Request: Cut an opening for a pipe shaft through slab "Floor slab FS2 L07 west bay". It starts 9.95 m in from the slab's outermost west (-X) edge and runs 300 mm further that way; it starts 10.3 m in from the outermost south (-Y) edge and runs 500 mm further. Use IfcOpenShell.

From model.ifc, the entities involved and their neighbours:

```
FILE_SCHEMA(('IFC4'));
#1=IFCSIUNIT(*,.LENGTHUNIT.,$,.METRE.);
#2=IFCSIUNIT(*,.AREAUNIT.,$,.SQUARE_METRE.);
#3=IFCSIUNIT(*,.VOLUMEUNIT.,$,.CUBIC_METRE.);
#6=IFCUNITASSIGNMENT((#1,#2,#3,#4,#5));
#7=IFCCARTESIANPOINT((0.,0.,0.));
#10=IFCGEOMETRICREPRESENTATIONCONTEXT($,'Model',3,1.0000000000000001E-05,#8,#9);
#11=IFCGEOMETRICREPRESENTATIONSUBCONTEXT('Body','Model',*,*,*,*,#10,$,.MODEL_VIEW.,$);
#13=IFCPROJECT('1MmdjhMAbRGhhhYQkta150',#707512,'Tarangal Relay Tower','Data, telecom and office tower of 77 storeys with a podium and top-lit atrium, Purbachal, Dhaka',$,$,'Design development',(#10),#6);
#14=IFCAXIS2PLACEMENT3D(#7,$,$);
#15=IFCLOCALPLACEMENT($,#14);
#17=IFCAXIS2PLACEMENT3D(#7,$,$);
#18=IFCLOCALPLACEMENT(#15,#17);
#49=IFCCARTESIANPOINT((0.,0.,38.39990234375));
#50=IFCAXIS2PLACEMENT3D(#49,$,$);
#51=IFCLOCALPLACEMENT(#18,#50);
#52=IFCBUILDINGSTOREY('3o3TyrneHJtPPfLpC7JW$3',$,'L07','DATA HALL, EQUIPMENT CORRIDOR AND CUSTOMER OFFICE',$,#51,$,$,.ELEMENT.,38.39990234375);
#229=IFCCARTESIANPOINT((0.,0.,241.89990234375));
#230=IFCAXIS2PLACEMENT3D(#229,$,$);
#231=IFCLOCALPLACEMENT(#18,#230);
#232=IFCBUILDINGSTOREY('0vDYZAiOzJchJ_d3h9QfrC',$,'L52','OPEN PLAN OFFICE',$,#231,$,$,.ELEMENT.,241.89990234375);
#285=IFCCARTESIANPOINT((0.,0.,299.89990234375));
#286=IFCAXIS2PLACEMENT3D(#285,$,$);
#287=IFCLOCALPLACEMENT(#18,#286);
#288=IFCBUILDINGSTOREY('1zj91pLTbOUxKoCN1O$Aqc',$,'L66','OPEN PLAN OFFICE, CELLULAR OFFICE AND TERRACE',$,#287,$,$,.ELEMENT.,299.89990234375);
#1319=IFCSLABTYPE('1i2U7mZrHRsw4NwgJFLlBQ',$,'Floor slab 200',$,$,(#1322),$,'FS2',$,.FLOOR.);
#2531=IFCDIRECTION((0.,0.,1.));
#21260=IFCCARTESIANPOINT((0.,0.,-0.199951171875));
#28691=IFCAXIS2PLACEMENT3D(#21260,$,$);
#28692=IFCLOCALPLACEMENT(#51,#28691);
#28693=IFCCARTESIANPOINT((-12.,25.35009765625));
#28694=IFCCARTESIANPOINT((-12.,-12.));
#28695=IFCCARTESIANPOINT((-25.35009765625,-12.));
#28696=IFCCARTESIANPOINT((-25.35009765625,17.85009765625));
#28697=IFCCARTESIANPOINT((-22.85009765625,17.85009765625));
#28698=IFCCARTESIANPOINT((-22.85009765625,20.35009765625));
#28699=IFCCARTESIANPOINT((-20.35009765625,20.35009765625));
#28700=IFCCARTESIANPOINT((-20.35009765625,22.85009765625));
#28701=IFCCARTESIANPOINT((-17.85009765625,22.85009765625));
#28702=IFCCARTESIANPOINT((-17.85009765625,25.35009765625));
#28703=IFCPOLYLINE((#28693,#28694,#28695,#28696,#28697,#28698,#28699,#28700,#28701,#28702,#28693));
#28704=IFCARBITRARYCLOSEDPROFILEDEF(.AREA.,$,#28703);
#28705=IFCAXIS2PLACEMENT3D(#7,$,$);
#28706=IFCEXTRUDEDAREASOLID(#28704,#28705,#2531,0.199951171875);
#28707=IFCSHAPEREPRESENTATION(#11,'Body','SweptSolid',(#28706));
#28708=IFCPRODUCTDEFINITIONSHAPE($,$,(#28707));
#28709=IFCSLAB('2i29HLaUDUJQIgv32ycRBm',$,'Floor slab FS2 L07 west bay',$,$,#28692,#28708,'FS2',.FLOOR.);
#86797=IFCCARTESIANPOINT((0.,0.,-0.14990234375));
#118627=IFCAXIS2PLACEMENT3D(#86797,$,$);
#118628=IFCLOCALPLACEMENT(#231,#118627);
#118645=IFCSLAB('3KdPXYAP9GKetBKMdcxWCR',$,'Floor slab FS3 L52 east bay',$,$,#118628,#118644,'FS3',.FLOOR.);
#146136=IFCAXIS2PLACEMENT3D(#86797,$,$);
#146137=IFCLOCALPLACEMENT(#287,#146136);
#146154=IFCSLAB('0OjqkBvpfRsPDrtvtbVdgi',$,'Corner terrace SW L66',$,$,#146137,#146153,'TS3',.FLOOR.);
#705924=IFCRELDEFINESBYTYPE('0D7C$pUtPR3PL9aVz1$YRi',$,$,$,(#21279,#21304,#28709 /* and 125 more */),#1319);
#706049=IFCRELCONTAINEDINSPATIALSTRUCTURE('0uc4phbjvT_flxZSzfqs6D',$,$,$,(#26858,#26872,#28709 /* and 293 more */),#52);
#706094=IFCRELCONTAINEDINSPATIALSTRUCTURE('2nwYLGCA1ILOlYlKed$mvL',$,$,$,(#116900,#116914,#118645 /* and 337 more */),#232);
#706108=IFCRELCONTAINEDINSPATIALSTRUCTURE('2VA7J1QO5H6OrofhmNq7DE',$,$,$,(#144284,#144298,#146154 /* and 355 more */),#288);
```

```python
import numpy as np
import ifcopenshell
import ifcopenshell.api.feature
import ifcopenshell.api.geometry
import ifcopenshell.api.root
import ifcopenshell.geom
import ifcopenshell.util.placement
import ifcopenshell.util.representation
import ifcopenshell.util.shape
import ifcopenshell.util.unit

model = ifcopenshell.open("model.ifc")
unit_scale = ifcopenshell.util.unit.calculate_unit_scale(model)
settings = ifcopenshell.geom.settings()


def volume(element):
    """Net volume in cubic metres, openings subtracted."""
    shape = ifcopenshell.geom.create_shape(settings, element)
    return ifcopenshell.util.shape.get_volume(shape.geometry)


slab = model.by_guid("2i29HLaUDUJQIgv32ycRBm")
before = volume(slab)

# Extent in the slab's own axes, in metres. The edges named are its -X and -Y sides.
slab_shape = ifcopenshell.geom.create_shape(settings, slab)
vertices = ifcopenshell.util.shape.get_vertices(slab_shape.geometry)
x_min, y_min, bottom = vertices.min(axis=0)
top = vertices[:, 2].max()

opening = ifcopenshell.api.root.create_entity(model, ifc_class="IfcOpeningElement", name="Pipe shaft opening", predefined_type="OPENING")
context = ifcopenshell.util.representation.get_context(model, "Model", "Body", "MODEL_VIEW")
width, depth = 0.3, 0.5
outline = [(0.0, 0.0), (width, 0.0), (width, depth), (0.0, depth), (0.0, 0.0)]
# Overshoot both faces by 50 mm so the cut is clean.
shape = ifcopenshell.api.geometry.add_slab_representation(
    model, context=context, depth=top - bottom + 0.1, polyline=outline
)
ifcopenshell.api.geometry.assign_representation(model, product=opening, representation=shape)

matrix = ifcopenshell.util.placement.get_local_placement(slab.ObjectPlacement)
matrix[:, 3] = matrix @ np.append(np.array([x_min + 9.95, y_min + 10.3, bottom - 0.05]) / unit_scale, 1.0)
ifcopenshell.api.geometry.edit_object_placement(model, product=opening, matrix=matrix, is_si=False)
ifcopenshell.api.feature.add_feature(model, feature=opening, element=slab)

after = volume(slab)

print(f"slab volume {before:.3f} -> {after:.3f} m3")

model.write("model_rev.ifc")
```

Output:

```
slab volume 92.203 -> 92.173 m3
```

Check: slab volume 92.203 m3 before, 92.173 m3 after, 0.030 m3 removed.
